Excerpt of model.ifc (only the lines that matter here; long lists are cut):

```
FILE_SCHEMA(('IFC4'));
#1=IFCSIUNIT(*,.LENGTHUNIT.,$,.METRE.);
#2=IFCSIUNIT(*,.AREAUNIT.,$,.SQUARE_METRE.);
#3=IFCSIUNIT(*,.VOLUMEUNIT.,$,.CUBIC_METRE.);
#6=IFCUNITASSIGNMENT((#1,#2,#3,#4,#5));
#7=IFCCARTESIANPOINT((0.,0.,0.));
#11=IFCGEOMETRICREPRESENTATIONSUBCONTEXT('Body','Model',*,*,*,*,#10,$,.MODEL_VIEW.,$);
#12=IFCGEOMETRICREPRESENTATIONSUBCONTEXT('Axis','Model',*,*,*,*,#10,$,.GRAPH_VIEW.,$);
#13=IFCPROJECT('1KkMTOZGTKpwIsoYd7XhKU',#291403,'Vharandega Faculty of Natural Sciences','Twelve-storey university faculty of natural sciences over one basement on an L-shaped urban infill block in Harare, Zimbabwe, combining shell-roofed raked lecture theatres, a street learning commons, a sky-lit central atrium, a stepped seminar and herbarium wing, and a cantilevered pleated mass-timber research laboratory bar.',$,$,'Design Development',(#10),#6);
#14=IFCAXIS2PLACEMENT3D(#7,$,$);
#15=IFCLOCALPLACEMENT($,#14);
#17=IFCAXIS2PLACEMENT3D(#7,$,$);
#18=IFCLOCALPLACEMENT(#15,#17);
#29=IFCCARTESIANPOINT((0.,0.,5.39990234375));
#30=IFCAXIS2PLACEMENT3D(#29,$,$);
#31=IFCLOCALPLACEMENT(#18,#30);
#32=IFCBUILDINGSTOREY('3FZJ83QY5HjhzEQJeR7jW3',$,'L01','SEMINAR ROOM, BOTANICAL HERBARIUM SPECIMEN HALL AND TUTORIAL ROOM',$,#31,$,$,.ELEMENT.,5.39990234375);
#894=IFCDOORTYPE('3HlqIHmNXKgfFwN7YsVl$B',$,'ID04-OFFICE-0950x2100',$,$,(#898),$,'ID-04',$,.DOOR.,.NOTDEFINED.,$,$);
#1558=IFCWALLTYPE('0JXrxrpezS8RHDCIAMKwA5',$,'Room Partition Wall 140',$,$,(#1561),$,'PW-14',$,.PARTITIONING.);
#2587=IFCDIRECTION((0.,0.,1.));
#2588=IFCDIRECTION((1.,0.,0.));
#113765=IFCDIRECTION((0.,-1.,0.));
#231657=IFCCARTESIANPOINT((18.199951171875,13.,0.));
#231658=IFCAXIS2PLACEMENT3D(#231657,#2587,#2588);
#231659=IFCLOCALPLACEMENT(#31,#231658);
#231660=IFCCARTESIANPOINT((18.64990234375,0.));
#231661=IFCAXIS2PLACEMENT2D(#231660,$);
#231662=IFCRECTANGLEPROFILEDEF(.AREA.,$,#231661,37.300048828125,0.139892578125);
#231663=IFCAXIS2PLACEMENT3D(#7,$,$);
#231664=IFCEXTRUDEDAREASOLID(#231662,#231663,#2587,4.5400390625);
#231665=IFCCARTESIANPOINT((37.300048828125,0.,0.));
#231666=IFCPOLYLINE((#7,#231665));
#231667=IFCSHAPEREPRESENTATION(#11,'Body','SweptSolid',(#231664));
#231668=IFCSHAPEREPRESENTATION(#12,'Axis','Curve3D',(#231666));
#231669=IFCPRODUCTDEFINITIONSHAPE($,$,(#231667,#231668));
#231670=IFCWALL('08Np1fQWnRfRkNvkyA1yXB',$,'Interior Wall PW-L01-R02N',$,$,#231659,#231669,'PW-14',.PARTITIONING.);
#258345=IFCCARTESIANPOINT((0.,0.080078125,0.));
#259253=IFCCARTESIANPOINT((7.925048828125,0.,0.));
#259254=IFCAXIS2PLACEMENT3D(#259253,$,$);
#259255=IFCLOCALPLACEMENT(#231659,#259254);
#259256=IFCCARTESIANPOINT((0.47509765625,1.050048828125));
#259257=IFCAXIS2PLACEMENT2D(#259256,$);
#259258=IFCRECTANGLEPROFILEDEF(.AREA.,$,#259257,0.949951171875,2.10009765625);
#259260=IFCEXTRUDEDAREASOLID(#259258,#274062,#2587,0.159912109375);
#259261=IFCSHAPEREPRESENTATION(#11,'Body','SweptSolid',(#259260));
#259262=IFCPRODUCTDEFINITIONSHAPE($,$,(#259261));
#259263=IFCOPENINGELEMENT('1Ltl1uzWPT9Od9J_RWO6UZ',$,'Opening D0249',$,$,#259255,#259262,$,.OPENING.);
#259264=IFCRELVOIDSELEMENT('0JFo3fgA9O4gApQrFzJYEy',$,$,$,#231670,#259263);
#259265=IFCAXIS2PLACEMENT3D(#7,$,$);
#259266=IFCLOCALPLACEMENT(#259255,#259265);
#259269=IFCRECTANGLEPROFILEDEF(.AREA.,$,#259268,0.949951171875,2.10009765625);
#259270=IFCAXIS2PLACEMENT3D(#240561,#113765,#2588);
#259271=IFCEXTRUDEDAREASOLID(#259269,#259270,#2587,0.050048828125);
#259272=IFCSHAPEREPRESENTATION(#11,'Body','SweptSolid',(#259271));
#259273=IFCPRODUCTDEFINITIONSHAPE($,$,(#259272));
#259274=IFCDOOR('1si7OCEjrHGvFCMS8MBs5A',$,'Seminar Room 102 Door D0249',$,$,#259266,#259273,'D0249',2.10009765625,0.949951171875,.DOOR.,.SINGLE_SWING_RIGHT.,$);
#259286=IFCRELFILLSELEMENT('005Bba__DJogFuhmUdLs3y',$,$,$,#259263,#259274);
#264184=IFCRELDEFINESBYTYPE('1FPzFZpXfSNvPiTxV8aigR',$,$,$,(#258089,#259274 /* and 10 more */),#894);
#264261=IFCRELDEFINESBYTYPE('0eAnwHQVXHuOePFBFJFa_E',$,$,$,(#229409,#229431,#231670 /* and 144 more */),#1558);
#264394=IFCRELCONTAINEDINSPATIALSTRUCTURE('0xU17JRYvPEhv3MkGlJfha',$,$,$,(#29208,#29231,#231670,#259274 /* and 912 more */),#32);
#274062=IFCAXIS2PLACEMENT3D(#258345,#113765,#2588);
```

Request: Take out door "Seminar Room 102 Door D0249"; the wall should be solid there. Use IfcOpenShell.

```python
import ifcopenshell
import ifcopenshell.api.feature
import ifcopenshell.api.root
import ifcopenshell.geom
import ifcopenshell.util.shape

model = ifcopenshell.open("model.ifc")
settings = ifcopenshell.geom.settings()


def volume(element):
    """Net volume in cubic metres, openings subtracted."""
    shape = ifcopenshell.geom.create_shape(settings, element)
    return ifcopenshell.util.shape.get_volume(shape.geometry)


door = model.by_guid("1si7OCEjrHGvFCMS8MBs5A")
opening = door.FillsVoids[0].RelatingOpeningElement
wall = opening.VoidsElements[0].RelatingBuildingElement
before = volume(wall)

ifcopenshell.api.root.remove_product(model, product=door)
ifcopenshell.api.feature.remove_feature(model, feature=opening)

after = volume(wall)

print(f"wall volume {before:.3f} -> {after:.3f} m3")

model.write("model_edited.ifc")
```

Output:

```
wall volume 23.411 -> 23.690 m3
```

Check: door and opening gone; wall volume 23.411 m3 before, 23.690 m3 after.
